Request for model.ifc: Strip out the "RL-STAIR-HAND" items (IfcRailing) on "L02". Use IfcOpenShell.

First a look at what the model holds.

```python
import ifcopenshell
import ifcopenshell.util.element

model = ifcopenshell.open("model.ifc")
print(model.schema)
storey = next(s for s in model.by_type("IfcBuildingStorey") if s.Name == "L02")
railings = [e for e in ifcopenshell.util.element.get_decomposition(storey) if e.is_a("IfcRailing")]
seen = {}
for e in railings:
    element_type = ifcopenshell.util.element.get_type(e)
    name = element_type.Name if element_type not in (None, e) else None
    seen[name] = seen.get(name, 0) + 1
for name, count in sorted(seen.items(), key=str):
    print(count, "x", name)
```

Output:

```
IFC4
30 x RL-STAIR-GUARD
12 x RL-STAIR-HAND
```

```python
import ifcopenshell
import ifcopenshell.api.root
import ifcopenshell.util.element

model = ifcopenshell.open("model.ifc")

storey = next(s for s in model.by_type("IfcBuildingStorey") if s.Name == "L02")
railings = [e for e in ifcopenshell.util.element.get_decomposition(storey) if e.is_a("IfcRailing")]
targets = [e for e in railings if (t := ifcopenshell.util.element.get_type(e)) not in (None, e) and t.Name == "RL-STAIR-HAND"]

for e in targets:
    ifcopenshell.api.root.remove_product(model, product=e)
print(len(targets), "removed")

model.write("model_edited.ifc")
```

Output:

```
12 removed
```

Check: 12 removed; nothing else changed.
